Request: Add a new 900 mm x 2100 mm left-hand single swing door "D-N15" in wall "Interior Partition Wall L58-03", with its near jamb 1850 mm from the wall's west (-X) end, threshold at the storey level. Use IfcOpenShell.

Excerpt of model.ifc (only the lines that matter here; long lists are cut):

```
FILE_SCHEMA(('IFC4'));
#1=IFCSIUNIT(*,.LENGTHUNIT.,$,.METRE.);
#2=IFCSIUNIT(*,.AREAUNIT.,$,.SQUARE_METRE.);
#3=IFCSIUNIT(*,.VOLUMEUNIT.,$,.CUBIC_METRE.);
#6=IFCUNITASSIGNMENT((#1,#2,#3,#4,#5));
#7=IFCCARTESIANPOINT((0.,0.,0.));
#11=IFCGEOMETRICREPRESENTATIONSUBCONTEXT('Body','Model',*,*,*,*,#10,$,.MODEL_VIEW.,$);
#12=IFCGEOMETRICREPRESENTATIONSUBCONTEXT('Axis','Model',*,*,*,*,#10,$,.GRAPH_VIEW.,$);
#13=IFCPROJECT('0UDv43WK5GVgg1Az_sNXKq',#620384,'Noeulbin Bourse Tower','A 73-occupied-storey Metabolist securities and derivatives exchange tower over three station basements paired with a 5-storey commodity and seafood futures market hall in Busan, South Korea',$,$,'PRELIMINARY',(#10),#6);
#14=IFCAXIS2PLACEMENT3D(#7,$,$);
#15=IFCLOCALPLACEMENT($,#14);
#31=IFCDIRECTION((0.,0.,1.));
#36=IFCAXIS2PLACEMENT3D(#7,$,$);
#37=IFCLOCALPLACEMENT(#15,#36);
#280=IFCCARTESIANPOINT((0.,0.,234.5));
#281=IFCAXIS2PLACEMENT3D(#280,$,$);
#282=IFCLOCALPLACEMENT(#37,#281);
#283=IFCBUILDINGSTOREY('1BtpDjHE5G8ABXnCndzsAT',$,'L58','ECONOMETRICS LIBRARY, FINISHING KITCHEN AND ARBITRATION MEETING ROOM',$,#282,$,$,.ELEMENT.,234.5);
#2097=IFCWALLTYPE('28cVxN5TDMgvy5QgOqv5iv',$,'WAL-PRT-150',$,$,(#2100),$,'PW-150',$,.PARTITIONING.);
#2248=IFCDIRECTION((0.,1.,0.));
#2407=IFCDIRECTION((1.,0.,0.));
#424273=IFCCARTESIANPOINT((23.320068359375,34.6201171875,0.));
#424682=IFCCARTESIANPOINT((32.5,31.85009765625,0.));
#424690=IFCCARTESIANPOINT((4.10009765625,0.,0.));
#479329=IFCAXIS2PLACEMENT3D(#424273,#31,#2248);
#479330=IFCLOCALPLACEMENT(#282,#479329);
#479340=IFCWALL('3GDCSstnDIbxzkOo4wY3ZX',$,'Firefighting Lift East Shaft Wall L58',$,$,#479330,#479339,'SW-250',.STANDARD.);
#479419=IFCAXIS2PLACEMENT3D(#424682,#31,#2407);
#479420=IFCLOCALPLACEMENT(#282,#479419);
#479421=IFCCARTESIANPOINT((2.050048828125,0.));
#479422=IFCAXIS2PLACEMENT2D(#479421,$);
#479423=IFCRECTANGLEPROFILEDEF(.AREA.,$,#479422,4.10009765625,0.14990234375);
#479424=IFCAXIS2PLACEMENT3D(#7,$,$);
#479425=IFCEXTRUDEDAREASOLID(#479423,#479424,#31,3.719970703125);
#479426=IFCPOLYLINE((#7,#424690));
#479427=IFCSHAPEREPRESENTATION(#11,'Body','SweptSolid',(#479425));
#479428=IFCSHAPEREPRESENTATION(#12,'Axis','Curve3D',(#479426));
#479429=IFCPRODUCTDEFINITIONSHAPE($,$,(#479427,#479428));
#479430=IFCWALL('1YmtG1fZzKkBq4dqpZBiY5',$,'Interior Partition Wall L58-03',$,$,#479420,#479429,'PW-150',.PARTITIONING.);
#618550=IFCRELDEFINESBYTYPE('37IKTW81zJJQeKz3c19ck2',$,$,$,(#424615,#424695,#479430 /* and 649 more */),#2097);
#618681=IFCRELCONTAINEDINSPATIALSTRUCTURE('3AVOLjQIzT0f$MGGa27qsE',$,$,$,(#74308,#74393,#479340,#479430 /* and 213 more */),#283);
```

```python
import numpy as np
import ifcopenshell
import ifcopenshell.api.feature
import ifcopenshell.api.geometry
import ifcopenshell.api.root
import ifcopenshell.api.spatial
import ifcopenshell.geom
import ifcopenshell.util.element
import ifcopenshell.util.placement
import ifcopenshell.util.representation
import ifcopenshell.util.shape
import ifcopenshell.util.unit

model = ifcopenshell.open("model.ifc")
unit_scale = ifcopenshell.util.unit.calculate_unit_scale(model)
settings = ifcopenshell.geom.settings()


def volume(element):
    """Net volume in cubic metres, openings subtracted."""
    shape = ifcopenshell.geom.create_shape(settings, element)
    return ifcopenshell.util.shape.get_volume(shape.geometry)


wall = model.by_guid("1YmtG1fZzKkBq4dqpZBiY5")
storey = ifcopenshell.util.element.get_container(wall, ifc_class="IfcBuildingStorey")
context = ifcopenshell.util.representation.get_context(model, "Model", "Body", "MODEL_VIEW")
before = volume(wall)

width, height, from_end, sill = 0.9, 2.1, 1.85, 0.0  # metres

# The wall runs along its own X axis, and the end named is its -X end.
wall_shape = ifcopenshell.geom.create_shape(settings, wall)
x, y, z = ifcopenshell.util.shape.get_vertices(wall_shape.geometry).T
start = x.min() + from_end
face, thickness = float(y.min()), float(y.max() - y.min())
wall_matrix = ifcopenshell.util.placement.get_local_placement(wall.ObjectPlacement)
level = ifcopenshell.util.placement.get_local_placement(storey.ObjectPlacement)[2, 3]


def in_wall(x, y):
    """Placement at x, y metres in the wall's axes, at sill height."""
    matrix = wall_matrix.copy()
    matrix[:, 3] = wall_matrix @ np.array([x / unit_scale, y / unit_scale, 0.0, 1.0])
    matrix[2, 3] = level + sill / unit_scale
    return matrix


# Opening: a box that overshoots both wall faces by 50 mm.
opening = ifcopenshell.api.root.create_entity(model, ifc_class="IfcOpeningElement", predefined_type="OPENING")
box = ifcopenshell.api.geometry.add_wall_representation(
    model, context=context, length=width, height=height, thickness=thickness + 0.1
)
ifcopenshell.api.geometry.assign_representation(model, product=opening, representation=box)
ifcopenshell.api.geometry.edit_object_placement(model, product=opening, matrix=in_wall(start, face - 0.05), is_si=False)
ifcopenshell.api.feature.add_feature(model, feature=opening, element=wall)

door = ifcopenshell.api.root.create_entity(model, ifc_class="IfcDoor", name="D-N15", predefined_type="DOOR")
door.OverallWidth, door.OverallHeight = width / unit_scale, height / unit_scale
door.OperationType = "SINGLE_SWING_LEFT"
body = ifcopenshell.api.geometry.add_door_representation(
    model,
    context=context,
    overall_width=door.OverallWidth,
    overall_height=door.OverallHeight,
    operation_type="SINGLE_SWING_LEFT",
    lining_properties={"LiningDepth": thickness / unit_scale, "ThresholdDepth": thickness / unit_scale},
)
ifcopenshell.api.geometry.assign_representation(model, product=door, representation=body)
ifcopenshell.api.spatial.assign_container(model, products=[door], relating_structure=storey)
ifcopenshell.api.feature.add_filling(model, opening=opening, element=door)

# The lining spans the wall, so the door starts at the wall face.
ifcopenshell.api.geometry.edit_object_placement(model, product=door, matrix=in_wall(start, face), is_si=False)

after = volume(wall)

print(f"wall volume {before:.3f} -> {after:.3f} m3")

model.write("model_edited.ifc")
```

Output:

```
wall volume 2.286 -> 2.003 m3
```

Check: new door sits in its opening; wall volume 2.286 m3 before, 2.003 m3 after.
